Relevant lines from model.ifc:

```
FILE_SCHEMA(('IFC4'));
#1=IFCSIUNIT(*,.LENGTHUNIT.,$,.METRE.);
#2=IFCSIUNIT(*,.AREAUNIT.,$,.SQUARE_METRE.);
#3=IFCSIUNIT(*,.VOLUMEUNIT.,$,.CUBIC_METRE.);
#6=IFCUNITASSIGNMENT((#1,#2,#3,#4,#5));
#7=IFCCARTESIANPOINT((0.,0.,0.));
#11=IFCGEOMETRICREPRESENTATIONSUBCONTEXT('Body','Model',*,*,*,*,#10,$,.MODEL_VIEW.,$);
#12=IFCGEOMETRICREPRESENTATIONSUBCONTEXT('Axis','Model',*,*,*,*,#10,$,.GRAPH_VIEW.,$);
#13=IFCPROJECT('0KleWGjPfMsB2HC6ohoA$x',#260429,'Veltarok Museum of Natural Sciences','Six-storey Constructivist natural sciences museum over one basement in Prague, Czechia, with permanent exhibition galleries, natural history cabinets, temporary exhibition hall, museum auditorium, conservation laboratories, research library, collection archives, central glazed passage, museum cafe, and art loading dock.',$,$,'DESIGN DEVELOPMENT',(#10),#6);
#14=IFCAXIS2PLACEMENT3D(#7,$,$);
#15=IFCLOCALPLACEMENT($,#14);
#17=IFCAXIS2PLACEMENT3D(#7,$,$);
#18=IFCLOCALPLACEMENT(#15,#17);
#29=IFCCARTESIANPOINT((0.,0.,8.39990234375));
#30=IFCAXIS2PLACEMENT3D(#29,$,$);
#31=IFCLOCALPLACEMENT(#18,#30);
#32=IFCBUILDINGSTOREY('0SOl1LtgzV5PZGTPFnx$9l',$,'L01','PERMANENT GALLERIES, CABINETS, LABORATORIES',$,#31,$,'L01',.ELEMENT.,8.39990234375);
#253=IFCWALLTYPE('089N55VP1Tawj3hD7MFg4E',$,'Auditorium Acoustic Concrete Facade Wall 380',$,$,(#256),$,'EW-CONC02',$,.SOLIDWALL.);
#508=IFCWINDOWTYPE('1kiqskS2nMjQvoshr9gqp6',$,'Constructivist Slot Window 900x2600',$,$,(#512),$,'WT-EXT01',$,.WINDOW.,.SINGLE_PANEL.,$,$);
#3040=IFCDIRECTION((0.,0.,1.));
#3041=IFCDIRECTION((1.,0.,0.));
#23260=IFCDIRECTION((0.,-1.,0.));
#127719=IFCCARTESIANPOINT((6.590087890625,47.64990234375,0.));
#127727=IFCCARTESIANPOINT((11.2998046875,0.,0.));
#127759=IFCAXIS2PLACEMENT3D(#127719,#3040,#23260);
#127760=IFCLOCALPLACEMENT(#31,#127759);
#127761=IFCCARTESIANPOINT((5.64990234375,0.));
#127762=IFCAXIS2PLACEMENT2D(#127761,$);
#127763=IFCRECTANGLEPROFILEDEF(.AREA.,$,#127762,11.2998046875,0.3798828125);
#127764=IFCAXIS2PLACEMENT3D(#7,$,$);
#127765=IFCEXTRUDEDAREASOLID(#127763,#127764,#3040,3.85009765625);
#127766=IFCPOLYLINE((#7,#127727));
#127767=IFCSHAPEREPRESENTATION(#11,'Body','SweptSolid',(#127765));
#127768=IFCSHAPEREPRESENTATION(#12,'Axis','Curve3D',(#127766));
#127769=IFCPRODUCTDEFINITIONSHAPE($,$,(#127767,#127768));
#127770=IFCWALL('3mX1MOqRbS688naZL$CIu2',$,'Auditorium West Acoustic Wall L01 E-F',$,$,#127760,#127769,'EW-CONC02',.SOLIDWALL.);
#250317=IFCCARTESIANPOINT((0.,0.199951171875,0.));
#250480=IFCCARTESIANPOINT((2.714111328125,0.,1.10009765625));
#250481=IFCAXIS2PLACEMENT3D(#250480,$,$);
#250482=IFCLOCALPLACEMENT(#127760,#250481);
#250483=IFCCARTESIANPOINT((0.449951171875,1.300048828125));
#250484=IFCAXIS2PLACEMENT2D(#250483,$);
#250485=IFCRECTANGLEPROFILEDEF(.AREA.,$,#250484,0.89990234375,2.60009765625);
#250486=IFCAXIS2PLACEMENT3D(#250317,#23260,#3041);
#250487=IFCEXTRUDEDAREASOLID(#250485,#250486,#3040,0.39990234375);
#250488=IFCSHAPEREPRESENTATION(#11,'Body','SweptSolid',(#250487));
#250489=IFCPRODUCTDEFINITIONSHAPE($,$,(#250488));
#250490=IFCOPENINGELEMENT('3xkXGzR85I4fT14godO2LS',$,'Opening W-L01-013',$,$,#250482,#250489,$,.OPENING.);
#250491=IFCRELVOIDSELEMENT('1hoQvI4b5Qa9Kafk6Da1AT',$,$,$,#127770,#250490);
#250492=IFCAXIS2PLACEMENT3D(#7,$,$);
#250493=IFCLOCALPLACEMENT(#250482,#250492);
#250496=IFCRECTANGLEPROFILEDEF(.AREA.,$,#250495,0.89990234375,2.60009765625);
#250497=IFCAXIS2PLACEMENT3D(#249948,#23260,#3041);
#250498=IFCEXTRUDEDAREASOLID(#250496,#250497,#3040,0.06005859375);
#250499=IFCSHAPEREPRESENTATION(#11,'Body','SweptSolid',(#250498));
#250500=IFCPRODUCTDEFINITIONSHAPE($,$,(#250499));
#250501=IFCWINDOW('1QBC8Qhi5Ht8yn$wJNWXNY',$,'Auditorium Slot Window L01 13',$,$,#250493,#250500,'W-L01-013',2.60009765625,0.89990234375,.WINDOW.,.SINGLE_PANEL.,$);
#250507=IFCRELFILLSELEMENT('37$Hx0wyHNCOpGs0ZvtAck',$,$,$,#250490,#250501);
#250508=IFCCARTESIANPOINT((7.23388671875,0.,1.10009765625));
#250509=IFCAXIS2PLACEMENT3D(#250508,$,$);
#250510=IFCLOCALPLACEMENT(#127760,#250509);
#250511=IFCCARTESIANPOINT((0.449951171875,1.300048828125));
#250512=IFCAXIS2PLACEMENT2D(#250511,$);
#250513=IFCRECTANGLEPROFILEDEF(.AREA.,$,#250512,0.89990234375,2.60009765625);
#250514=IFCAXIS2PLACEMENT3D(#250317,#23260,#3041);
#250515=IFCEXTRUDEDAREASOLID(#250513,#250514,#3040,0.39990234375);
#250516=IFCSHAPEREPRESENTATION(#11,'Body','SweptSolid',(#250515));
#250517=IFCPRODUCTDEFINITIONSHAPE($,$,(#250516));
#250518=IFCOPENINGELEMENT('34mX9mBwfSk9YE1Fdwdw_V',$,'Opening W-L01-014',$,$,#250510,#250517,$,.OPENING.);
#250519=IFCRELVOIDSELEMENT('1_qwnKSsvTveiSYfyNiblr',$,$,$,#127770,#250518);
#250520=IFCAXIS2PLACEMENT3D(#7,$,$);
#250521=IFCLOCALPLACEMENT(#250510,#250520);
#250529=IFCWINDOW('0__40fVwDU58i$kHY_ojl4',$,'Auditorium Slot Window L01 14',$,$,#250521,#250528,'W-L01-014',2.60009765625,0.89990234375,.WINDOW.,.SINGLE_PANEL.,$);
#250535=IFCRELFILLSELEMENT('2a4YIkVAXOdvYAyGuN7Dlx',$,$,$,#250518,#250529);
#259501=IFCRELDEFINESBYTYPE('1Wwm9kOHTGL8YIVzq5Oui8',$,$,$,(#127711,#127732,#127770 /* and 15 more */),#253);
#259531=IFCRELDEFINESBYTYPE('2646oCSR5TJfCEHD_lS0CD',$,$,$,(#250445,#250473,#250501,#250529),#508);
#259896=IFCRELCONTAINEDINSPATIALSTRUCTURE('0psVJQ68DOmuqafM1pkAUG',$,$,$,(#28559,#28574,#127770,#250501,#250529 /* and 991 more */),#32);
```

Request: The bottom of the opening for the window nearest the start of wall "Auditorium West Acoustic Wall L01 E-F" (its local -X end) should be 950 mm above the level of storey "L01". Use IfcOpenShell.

```python
import numpy as np
import ifcopenshell
import ifcopenshell.api.geometry
import ifcopenshell.geom
import ifcopenshell.util.element
import ifcopenshell.util.placement
import ifcopenshell.util.shape
import ifcopenshell.util.unit

model = ifcopenshell.open("model.ifc")
unit_scale = ifcopenshell.util.unit.calculate_unit_scale(model)

window = model.by_guid("1QBC8Qhi5Ht8yn$wJNWXNY")
opening = window.FillsVoids[0].RelatingOpeningElement
storey = ifcopenshell.util.element.get_container(window, ifc_class="IfcBuildingStorey")
level = ifcopenshell.util.placement.get_local_placement(storey.ObjectPlacement)[2, 3]

# The opening's origin need not be at the sill, so measure its lowest point.
shape = ifcopenshell.geom.create_shape(ifcopenshell.geom.settings(), opening)
bottom = ifcopenshell.util.shape.get_shape_bottom_elevation(shape, shape.geometry) / unit_scale
dz = level + 0.95 / unit_scale - bottom

shift = np.array([0.0, 0.0, dz])
# The window is placed relative to its opening, so it follows when the opening moves.
matrix = ifcopenshell.util.placement.get_local_placement(opening.ObjectPlacement)
matrix[:3, 3] += shift
ifcopenshell.api.geometry.edit_object_placement(
    model, product=opening, matrix=matrix, is_si=False, should_transform_children=True
)

print(f"moved by {dz * unit_scale:+.3f} m")

model.write("model_v2.ifc")
```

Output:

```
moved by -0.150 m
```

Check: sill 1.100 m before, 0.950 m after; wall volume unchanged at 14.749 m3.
